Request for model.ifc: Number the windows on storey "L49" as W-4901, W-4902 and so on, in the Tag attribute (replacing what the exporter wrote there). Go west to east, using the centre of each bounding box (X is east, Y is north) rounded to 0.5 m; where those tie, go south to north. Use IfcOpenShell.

First a look at what the model holds.

```python
import ifcopenshell
import ifcopenshell.util.element
import ifcopenshell.util.placement

model = ifcopenshell.open("model.ifc")
print(model.schema)
storey = next(s for s in model.by_type("IfcBuildingStorey") if s.Name == "L49")
windows = [e for e in ifcopenshell.util.element.get_decomposition(storey) if e.is_a("IfcWindow")]
for e in sorted(windows, key=lambda e: e.id()):
    origin = ifcopenshell.util.placement.get_local_placement(e.ObjectPlacement)[:3, 3]
    print(e.id(), e.Tag, e.Name, origin.round(2) + 0.0, sep=" | ")
```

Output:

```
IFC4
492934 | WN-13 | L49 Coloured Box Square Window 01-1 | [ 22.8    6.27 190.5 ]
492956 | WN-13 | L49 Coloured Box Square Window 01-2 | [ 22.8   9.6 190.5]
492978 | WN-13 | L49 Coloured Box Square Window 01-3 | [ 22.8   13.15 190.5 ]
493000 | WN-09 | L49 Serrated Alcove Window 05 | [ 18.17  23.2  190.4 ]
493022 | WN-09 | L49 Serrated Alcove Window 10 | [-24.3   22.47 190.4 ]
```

```python
import ifcopenshell
import ifcopenshell.geom
import ifcopenshell.util.element
import ifcopenshell.util.shape

model = ifcopenshell.open("model.ifc")
settings = ifcopenshell.geom.settings()
settings.set("use-world-coords", True)


def centre(element):
    shape = ifcopenshell.geom.create_shape(settings, element)
    return ifcopenshell.util.shape.get_bbox_centroid(shape.geometry)


storey = next(s for s in model.by_type("IfcBuildingStorey") if s.Name == "L49")
windows = [e for e in ifcopenshell.util.element.get_decomposition(storey) if e.is_a("IfcWindow")]

# Insertion points can sit at a corner or the storey origin, so sort by the geometry (in metres).
centres = {e: centre(e) for e in windows}
windows.sort(key=lambda e: (round(centres[e][0] / 0.5), centres[e][1]))

for i, e in enumerate(windows, start=1):
    number = f"W-49{i:02d}"
    e.Tag = number
    print(e.id(), number)

model.write("model-out.ifc")
```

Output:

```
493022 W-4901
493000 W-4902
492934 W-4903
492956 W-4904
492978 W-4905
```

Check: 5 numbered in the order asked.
